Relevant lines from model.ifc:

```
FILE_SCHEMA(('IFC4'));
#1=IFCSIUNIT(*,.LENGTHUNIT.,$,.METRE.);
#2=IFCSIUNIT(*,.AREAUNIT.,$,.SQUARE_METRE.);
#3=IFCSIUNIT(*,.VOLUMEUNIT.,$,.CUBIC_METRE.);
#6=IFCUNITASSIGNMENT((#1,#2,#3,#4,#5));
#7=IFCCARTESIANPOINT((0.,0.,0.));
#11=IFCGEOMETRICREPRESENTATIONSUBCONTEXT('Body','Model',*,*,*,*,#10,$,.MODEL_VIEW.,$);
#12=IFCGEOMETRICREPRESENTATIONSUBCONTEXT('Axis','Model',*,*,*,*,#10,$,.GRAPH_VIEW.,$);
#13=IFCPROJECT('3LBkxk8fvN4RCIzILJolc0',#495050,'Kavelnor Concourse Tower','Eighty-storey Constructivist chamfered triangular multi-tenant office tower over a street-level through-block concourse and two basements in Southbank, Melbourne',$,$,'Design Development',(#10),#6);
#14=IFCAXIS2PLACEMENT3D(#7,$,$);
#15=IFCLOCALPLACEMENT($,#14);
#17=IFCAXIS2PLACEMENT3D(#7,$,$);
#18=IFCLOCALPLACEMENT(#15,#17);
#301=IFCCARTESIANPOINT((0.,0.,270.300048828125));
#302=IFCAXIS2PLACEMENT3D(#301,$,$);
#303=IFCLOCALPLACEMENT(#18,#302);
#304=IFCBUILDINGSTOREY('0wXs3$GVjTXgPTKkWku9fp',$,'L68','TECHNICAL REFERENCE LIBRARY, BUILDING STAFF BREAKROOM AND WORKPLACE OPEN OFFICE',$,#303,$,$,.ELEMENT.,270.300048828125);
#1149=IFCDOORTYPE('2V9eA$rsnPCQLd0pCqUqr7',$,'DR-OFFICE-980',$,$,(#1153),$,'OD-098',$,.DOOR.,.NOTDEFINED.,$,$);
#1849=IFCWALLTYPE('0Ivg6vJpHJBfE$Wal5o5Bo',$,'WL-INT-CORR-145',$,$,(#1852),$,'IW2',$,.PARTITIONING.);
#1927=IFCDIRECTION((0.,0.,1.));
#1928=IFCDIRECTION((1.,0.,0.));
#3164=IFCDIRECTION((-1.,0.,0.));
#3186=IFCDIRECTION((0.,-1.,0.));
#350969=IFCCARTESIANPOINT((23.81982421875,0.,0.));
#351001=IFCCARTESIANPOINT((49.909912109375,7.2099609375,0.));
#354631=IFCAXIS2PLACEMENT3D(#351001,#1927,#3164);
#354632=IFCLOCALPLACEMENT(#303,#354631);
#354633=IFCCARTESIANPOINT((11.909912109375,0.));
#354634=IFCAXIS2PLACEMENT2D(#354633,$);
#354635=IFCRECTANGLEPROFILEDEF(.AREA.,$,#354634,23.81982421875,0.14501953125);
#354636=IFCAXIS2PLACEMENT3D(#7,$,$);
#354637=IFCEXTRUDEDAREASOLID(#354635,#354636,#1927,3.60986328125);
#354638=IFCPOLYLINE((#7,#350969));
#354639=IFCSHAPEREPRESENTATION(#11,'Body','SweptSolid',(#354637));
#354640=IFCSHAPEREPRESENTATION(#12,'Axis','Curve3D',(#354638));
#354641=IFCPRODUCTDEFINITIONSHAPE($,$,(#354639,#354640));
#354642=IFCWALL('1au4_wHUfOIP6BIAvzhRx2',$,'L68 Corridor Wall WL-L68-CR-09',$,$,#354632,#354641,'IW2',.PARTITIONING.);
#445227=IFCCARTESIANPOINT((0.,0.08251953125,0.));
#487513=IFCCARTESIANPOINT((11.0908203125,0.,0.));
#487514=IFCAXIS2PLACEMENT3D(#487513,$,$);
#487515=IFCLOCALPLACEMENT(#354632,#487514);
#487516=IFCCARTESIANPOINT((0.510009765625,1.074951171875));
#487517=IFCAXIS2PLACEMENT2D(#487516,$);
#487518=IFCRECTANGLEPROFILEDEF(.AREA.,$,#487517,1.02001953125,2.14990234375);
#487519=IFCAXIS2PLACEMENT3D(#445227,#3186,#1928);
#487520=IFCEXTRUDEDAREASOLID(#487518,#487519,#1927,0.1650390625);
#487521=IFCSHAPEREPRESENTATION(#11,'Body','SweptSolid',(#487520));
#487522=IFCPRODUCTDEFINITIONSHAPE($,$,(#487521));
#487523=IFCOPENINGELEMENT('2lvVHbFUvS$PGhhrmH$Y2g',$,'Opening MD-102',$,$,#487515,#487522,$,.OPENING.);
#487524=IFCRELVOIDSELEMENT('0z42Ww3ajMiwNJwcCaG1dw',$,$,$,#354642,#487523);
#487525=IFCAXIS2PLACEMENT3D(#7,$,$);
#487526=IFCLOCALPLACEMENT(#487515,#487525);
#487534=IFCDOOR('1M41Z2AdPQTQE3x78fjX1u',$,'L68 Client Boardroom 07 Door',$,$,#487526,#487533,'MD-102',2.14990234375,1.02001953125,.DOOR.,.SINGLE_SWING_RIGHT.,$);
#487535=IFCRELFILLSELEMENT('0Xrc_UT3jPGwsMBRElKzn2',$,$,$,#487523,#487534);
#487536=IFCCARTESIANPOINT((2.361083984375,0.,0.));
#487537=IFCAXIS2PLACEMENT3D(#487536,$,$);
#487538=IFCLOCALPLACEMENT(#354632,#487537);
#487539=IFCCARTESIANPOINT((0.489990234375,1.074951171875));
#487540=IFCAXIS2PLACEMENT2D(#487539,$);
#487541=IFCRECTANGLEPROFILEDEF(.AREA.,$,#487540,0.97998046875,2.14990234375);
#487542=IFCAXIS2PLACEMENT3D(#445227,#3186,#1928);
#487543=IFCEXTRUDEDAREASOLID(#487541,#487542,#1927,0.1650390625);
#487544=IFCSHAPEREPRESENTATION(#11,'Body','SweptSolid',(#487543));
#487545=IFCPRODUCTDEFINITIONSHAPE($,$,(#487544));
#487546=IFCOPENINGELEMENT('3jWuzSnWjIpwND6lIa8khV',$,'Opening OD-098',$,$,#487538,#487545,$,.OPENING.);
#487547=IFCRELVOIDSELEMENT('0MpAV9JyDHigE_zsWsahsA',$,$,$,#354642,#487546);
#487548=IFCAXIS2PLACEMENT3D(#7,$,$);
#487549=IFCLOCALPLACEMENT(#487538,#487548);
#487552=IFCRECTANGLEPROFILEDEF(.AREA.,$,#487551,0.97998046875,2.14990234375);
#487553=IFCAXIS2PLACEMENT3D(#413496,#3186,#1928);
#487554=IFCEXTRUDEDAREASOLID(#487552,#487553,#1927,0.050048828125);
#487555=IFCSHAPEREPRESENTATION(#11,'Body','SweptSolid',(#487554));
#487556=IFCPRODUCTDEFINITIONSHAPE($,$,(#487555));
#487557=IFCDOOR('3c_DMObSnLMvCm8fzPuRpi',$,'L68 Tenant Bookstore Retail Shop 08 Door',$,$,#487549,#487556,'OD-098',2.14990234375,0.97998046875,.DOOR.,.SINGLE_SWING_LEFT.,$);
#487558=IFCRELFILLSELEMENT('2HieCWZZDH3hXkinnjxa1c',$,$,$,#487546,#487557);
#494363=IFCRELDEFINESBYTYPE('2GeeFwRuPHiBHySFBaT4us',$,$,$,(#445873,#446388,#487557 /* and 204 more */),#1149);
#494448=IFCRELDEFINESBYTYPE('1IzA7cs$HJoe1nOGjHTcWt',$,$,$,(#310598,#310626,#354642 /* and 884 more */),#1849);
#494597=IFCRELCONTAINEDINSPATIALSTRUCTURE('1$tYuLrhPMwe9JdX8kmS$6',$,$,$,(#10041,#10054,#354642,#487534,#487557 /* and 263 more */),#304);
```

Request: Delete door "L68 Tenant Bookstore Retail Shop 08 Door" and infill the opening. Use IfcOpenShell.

```python
import ifcopenshell
import ifcopenshell.api.feature
import ifcopenshell.api.root
import ifcopenshell.geom
import ifcopenshell.util.shape

model = ifcopenshell.open("model.ifc")
settings = ifcopenshell.geom.settings()


def volume(element):
    """Net volume in cubic metres, openings subtracted."""
    shape = ifcopenshell.geom.create_shape(settings, element)
    return ifcopenshell.util.shape.get_volume(shape.geometry)


door = model.by_guid("3c_DMObSnLMvCm8fzPuRpi")
opening = door.FillsVoids[0].RelatingOpeningElement
wall = opening.VoidsElements[0].RelatingBuildingElement
before = volume(wall)

ifcopenshell.api.root.remove_product(model, product=door)
ifcopenshell.api.feature.remove_feature(model, feature=opening)

after = volume(wall)

print(f"wall volume {before:.3f} -> {after:.3f} m3")

model.write("model_updated.ifc")
```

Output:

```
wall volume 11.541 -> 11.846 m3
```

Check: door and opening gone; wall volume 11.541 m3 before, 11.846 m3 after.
